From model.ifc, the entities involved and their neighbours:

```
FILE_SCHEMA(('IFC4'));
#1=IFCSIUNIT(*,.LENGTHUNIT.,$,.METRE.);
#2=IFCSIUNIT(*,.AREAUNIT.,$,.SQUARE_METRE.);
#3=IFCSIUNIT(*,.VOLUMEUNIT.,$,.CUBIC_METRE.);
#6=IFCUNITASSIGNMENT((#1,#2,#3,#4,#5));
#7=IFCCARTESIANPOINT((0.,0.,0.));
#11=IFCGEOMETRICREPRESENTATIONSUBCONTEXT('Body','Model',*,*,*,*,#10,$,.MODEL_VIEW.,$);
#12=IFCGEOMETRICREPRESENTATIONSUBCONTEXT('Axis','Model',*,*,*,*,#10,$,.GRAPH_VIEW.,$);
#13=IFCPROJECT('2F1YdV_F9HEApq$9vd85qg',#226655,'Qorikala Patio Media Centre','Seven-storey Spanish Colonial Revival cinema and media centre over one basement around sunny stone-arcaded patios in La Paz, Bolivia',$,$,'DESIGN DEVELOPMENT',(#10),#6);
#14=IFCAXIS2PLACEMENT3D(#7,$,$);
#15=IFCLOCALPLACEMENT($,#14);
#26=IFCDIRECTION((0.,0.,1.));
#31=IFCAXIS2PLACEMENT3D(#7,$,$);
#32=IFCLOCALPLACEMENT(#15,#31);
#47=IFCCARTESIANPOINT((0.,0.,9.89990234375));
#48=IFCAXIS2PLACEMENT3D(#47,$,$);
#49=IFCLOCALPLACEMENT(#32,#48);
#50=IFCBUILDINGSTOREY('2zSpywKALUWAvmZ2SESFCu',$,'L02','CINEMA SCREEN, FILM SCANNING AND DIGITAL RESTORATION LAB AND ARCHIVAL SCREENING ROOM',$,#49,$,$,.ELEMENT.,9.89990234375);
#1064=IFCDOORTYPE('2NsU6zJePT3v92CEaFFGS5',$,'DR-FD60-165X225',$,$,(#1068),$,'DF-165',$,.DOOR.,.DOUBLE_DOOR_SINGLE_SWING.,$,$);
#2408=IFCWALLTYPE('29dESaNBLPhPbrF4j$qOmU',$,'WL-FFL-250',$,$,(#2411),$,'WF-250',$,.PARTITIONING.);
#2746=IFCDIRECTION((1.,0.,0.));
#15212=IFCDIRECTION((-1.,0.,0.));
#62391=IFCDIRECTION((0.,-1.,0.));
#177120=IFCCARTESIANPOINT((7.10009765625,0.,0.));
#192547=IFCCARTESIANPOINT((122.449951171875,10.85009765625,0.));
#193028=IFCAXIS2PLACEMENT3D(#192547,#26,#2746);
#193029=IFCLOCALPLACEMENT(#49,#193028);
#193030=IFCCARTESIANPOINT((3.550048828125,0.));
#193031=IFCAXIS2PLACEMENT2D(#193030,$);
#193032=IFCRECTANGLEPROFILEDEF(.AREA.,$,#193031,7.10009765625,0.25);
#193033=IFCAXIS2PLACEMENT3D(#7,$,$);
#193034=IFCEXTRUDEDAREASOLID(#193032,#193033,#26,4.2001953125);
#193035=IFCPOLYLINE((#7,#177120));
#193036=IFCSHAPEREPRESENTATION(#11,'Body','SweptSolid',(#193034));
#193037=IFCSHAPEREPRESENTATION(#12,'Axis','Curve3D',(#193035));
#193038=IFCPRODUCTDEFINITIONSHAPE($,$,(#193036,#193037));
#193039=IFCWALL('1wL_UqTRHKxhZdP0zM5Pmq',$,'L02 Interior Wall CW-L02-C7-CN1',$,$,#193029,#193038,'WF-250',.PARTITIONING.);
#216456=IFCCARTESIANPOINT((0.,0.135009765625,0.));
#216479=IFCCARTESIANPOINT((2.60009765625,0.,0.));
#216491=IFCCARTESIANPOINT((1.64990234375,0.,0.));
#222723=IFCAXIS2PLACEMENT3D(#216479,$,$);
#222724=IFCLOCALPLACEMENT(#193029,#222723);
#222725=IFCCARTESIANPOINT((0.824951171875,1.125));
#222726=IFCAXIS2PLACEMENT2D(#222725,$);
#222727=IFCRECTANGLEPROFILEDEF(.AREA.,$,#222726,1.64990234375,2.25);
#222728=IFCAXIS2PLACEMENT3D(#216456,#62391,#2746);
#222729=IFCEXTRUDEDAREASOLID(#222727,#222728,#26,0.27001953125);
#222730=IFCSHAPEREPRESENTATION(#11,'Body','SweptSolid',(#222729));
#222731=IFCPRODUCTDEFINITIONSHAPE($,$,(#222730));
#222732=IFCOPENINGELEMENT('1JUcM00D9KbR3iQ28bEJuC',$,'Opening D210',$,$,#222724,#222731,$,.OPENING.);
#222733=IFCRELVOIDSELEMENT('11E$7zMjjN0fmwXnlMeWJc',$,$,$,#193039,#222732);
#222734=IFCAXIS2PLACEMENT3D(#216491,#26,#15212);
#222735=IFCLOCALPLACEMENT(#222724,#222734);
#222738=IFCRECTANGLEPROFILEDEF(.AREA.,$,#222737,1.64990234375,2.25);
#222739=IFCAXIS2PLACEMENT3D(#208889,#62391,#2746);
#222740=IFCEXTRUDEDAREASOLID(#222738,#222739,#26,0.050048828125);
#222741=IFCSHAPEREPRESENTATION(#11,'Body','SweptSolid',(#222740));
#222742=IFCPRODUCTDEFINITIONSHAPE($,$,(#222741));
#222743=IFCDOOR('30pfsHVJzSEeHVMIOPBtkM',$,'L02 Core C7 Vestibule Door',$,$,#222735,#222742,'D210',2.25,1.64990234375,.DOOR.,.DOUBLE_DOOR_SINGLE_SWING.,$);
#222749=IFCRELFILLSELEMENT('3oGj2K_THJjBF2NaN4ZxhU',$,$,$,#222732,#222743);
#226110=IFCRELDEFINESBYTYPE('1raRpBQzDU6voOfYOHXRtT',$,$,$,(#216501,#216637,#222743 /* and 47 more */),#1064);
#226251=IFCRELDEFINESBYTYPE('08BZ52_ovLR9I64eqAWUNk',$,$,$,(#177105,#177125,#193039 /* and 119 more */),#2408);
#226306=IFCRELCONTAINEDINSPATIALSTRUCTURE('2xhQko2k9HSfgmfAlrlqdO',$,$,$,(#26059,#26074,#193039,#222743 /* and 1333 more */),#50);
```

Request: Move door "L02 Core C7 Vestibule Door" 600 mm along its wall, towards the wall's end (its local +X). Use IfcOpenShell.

```python
import ifcopenshell
import ifcopenshell.api.geometry
import ifcopenshell.util.placement
import ifcopenshell.util.unit

model = ifcopenshell.open("model.ifc")
unit_scale = ifcopenshell.util.unit.calculate_unit_scale(model)

door = model.by_id(222743)
opening = door.FillsVoids[0].RelatingOpeningElement
wall = opening.VoidsElements[0].RelatingBuildingElement

wall_matrix = ifcopenshell.util.placement.get_local_placement(wall.ObjectPlacement)
shift = wall_matrix[:3, 0] * 0.6 / unit_scale
before = ifcopenshell.util.placement.get_local_placement(door.ObjectPlacement)[:3, 3].copy()

# The door is placed relative to its opening, so it follows when the opening moves.
matrix = ifcopenshell.util.placement.get_local_placement(opening.ObjectPlacement)
matrix[:3, 3] += shift
ifcopenshell.api.geometry.edit_object_placement(
    model, product=opening, matrix=matrix, is_si=False, should_transform_children=True
)

after = ifcopenshell.util.placement.get_local_placement(door.ObjectPlacement)[:3, 3]
print("door moved by", (after - before).round(3) + 0.0)

model.write("model_edited.ifc")
```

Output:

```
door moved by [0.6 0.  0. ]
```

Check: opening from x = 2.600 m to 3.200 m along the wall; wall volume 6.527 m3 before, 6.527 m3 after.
